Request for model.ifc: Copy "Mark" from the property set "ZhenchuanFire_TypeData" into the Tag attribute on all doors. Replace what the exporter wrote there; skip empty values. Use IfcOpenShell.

First a look at what the model holds.

```python
import ifcopenshell
import ifcopenshell.util.element

model = ifcopenshell.open("model.ifc")
print(model.schema)
doors = model.by_type("IfcDoor")
print(len(doors), "doors")
for e in doors[:8]:
    source = ifcopenshell.util.element.get_pset(e, "ZhenchuanFire_TypeData", "Mark")
    target = e.Tag
    print(e.id(), repr(source), repr(target), sep=" | ")
```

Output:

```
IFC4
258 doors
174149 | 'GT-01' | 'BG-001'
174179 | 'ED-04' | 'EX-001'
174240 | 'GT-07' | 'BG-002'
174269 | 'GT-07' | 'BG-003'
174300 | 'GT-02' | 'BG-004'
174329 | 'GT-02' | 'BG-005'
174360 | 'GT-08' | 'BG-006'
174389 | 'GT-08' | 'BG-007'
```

```python
import ifcopenshell
import ifcopenshell.util.element

model = ifcopenshell.open("model.ifc")

count = 0
for e in model.by_type("IfcDoor"):
    value = ifcopenshell.util.element.get_pset(e, "ZhenchuanFire_TypeData", "Mark")
    current = e.Tag
    if not value or not value.strip() or current == value:
        continue
    e.Tag = value
    count += 1

print(count, "doors updated")

model.write("model_updated.ifc")
```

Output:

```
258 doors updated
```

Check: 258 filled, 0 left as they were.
